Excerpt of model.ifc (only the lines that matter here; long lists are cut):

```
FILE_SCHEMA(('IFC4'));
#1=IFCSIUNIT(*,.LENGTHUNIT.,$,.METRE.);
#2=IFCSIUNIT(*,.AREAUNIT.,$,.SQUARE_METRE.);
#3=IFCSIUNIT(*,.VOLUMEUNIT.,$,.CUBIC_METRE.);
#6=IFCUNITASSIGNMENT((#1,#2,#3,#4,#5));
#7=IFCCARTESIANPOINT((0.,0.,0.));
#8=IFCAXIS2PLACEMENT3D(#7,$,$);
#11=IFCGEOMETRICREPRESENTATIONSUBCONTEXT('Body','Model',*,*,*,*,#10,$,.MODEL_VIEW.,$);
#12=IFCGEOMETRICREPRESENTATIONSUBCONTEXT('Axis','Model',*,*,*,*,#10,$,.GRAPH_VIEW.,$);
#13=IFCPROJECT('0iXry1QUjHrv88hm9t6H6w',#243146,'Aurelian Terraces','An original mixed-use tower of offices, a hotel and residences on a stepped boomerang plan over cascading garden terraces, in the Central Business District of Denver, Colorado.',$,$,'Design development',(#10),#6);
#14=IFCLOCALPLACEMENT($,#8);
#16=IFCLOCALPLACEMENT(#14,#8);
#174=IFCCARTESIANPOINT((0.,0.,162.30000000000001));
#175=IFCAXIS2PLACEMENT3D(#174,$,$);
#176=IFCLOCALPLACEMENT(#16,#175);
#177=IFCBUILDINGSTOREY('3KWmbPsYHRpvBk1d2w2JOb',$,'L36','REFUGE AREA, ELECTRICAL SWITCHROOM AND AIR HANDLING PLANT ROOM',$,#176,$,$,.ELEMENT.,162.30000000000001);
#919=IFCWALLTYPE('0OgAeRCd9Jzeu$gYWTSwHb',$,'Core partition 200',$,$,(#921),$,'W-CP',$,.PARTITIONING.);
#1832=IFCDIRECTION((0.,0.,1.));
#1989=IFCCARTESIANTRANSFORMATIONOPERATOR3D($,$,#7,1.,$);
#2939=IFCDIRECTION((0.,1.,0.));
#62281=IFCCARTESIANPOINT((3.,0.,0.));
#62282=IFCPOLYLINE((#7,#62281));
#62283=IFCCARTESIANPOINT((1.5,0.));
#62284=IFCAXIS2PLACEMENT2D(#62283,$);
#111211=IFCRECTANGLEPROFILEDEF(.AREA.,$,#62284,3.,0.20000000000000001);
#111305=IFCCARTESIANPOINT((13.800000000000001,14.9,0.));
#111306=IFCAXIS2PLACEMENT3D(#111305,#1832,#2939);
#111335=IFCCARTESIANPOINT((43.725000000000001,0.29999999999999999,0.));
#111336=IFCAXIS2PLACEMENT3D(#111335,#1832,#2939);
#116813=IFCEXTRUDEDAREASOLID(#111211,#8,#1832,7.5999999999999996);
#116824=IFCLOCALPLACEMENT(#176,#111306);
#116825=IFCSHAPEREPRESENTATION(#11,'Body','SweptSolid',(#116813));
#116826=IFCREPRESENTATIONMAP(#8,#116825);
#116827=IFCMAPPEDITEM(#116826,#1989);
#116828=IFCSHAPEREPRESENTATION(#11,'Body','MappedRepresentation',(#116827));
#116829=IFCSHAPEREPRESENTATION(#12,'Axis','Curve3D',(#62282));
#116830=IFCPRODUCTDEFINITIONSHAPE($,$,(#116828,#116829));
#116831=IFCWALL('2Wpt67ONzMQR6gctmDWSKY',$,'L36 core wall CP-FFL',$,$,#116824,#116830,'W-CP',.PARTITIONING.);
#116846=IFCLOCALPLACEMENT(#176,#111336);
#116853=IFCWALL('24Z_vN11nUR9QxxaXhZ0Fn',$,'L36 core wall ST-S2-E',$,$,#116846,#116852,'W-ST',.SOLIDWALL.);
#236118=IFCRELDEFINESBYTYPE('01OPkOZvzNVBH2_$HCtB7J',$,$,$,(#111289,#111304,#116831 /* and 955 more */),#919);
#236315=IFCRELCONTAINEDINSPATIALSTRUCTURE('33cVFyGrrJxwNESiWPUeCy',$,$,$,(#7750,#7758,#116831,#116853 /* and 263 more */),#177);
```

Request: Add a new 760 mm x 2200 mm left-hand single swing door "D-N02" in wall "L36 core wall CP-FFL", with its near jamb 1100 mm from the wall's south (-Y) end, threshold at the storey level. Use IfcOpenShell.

```python
import numpy as np
import ifcopenshell
import ifcopenshell.api.feature
import ifcopenshell.api.geometry
import ifcopenshell.api.root
import ifcopenshell.api.spatial
import ifcopenshell.geom
import ifcopenshell.util.element
import ifcopenshell.util.placement
import ifcopenshell.util.representation
import ifcopenshell.util.shape
import ifcopenshell.util.unit

model = ifcopenshell.open("model.ifc")
unit_scale = ifcopenshell.util.unit.calculate_unit_scale(model)
settings = ifcopenshell.geom.settings()


def volume(element):
    """Net volume in cubic metres, openings subtracted."""
    shape = ifcopenshell.geom.create_shape(settings, element)
    return ifcopenshell.util.shape.get_volume(shape.geometry)


wall = model.by_guid("2Wpt67ONzMQR6gctmDWSKY")
storey = ifcopenshell.util.element.get_container(wall, ifc_class="IfcBuildingStorey")
context = ifcopenshell.util.representation.get_context(model, "Model", "Body", "MODEL_VIEW")
before = volume(wall)

width, height, from_end, sill = 0.76, 2.2, 1.1, 0.0  # metres

# The wall runs along its own X axis, and the end named is its -X end.
wall_shape = ifcopenshell.geom.create_shape(settings, wall)
x, y, z = ifcopenshell.util.shape.get_vertices(wall_shape.geometry).T
start = x.min() + from_end
face, thickness = float(y.min()), float(y.max() - y.min())
wall_matrix = ifcopenshell.util.placement.get_local_placement(wall.ObjectPlacement)
level = ifcopenshell.util.placement.get_local_placement(storey.ObjectPlacement)[2, 3]


def in_wall(x, y):
    """Placement at x, y metres in the wall's axes, at sill height."""
    matrix = wall_matrix.copy()
    matrix[:, 3] = wall_matrix @ np.array([x / unit_scale, y / unit_scale, 0.0, 1.0])
    matrix[2, 3] = level + sill / unit_scale
    return matrix


# Opening: a box that overshoots both wall faces by 50 mm.
opening = ifcopenshell.api.root.create_entity(model, ifc_class="IfcOpeningElement", predefined_type="OPENING")
box = ifcopenshell.api.geometry.add_wall_representation(
    model, context=context, length=width, height=height, thickness=thickness + 0.1
)
ifcopenshell.api.geometry.assign_representation(model, product=opening, representation=box)
ifcopenshell.api.geometry.edit_object_placement(model, product=opening, matrix=in_wall(start, face - 0.05), is_si=False)
ifcopenshell.api.feature.add_feature(model, feature=opening, element=wall)

door = ifcopenshell.api.root.create_entity(model, ifc_class="IfcDoor", name="D-N02", predefined_type="DOOR")
door.OverallWidth, door.OverallHeight = width / unit_scale, height / unit_scale
door.OperationType = "SINGLE_SWING_LEFT"
body = ifcopenshell.api.geometry.add_door_representation(
    model,
    context=context,
    overall_width=door.OverallWidth,
    overall_height=door.OverallHeight,
    operation_type="SINGLE_SWING_LEFT",
    lining_properties={"LiningDepth": thickness / unit_scale, "ThresholdDepth": thickness / unit_scale},
)
ifcopenshell.api.geometry.assign_representation(model, product=door, representation=body)
ifcopenshell.api.spatial.assign_container(model, products=[door], relating_structure=storey)
ifcopenshell.api.feature.add_filling(model, opening=opening, element=door)

# The lining spans the wall, so the door starts at the wall face.
ifcopenshell.api.geometry.edit_object_placement(model, product=door, matrix=in_wall(start, face), is_si=False)

after = volume(wall)

print(f"wall volume {before:.3f} -> {after:.3f} m3")

model.write("model_v2.ifc")
```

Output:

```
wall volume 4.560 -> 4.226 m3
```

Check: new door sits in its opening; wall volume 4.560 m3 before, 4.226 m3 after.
